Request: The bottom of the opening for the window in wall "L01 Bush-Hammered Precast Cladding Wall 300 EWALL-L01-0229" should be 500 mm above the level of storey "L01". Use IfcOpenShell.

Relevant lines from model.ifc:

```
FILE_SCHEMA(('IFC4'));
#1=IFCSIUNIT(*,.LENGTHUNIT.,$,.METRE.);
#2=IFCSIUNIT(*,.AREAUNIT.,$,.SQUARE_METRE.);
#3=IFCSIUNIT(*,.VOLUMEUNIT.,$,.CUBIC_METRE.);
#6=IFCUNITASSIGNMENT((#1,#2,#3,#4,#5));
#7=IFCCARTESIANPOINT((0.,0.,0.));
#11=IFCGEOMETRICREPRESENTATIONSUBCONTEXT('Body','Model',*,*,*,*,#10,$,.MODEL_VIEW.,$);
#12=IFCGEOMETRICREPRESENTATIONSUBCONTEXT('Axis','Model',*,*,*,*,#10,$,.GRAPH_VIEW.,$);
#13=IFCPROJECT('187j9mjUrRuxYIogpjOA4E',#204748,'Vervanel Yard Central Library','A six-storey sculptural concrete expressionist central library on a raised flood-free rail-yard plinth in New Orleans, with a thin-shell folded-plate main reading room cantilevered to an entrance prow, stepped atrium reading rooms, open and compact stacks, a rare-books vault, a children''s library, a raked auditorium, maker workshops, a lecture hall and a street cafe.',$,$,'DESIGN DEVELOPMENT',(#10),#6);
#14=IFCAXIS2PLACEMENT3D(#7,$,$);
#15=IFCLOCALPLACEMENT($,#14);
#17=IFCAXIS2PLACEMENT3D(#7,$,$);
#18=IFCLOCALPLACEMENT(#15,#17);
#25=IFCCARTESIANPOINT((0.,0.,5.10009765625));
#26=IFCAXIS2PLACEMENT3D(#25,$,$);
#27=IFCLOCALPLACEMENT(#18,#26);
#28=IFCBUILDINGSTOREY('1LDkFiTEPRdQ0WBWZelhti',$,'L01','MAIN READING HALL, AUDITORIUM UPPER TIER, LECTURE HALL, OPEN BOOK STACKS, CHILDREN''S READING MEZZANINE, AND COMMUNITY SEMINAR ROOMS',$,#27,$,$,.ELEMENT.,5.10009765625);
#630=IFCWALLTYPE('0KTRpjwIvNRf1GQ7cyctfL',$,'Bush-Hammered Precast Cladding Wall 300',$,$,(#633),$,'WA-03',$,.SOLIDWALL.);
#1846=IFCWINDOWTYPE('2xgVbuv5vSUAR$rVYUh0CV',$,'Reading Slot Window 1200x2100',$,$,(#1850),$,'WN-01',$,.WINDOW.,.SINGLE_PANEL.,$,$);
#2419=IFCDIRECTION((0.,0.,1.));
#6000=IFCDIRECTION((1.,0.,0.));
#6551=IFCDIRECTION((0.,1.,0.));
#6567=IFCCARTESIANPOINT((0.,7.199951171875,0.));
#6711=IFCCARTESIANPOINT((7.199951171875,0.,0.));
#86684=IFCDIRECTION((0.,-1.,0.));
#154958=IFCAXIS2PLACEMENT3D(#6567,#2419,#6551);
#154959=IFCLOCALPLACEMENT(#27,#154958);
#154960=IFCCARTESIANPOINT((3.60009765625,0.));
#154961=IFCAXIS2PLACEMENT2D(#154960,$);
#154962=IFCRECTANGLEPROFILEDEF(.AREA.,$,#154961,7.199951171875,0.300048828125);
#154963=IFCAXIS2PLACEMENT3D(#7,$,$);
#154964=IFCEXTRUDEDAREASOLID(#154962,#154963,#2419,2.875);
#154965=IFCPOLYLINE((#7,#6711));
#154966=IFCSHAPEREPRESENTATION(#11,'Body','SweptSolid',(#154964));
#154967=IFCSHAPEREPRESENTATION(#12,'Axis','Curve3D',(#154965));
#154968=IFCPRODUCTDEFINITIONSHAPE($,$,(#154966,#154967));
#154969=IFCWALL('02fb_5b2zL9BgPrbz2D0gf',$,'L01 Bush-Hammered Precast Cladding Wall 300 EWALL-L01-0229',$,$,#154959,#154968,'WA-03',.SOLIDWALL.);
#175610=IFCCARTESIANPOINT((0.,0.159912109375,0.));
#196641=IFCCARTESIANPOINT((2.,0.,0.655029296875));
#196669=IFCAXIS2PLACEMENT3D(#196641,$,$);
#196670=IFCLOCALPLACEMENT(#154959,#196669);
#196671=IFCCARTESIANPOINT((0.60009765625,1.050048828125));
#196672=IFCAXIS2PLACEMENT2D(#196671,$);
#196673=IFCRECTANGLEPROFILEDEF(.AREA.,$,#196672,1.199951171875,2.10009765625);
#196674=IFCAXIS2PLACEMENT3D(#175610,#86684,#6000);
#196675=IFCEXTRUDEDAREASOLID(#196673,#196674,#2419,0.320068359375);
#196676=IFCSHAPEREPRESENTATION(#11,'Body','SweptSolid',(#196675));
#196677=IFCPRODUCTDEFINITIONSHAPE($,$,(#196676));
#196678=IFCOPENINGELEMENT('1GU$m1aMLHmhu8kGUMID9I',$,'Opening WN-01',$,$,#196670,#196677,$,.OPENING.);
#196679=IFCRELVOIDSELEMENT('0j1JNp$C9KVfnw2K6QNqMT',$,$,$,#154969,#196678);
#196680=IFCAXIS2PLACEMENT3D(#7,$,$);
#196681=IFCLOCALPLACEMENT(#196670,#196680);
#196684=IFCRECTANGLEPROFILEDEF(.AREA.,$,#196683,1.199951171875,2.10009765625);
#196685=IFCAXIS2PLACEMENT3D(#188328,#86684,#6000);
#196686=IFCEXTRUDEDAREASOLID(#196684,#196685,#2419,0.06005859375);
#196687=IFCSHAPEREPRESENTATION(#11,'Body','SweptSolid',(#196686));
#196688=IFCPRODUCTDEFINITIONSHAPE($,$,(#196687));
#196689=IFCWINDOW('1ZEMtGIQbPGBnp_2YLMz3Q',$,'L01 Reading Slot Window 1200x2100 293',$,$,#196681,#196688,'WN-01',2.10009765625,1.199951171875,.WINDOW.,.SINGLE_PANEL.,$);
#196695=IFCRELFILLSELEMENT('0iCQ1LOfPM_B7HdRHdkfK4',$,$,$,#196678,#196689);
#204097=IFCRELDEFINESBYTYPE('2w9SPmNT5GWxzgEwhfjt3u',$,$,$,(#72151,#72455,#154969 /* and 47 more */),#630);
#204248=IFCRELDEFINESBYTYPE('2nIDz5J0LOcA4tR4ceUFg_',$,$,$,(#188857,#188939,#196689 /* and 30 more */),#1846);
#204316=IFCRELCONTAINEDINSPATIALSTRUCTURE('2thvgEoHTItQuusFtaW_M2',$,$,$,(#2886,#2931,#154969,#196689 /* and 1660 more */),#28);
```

```python
import numpy as np
import ifcopenshell
import ifcopenshell.api.geometry
import ifcopenshell.geom
import ifcopenshell.util.element
import ifcopenshell.util.placement
import ifcopenshell.util.shape
import ifcopenshell.util.unit

model = ifcopenshell.open("model.ifc")
unit_scale = ifcopenshell.util.unit.calculate_unit_scale(model)

window = model.by_guid("1ZEMtGIQbPGBnp_2YLMz3Q")
opening = window.FillsVoids[0].RelatingOpeningElement
storey = ifcopenshell.util.element.get_container(window, ifc_class="IfcBuildingStorey")
level = ifcopenshell.util.placement.get_local_placement(storey.ObjectPlacement)[2, 3]

# The opening's origin need not be at the sill, so measure its lowest point.
shape = ifcopenshell.geom.create_shape(ifcopenshell.geom.settings(), opening)
bottom = ifcopenshell.util.shape.get_shape_bottom_elevation(shape, shape.geometry) / unit_scale
dz = level + 0.5 / unit_scale - bottom

shift = np.array([0.0, 0.0, dz])
# The window is placed relative to its opening, so it follows when the opening moves.
matrix = ifcopenshell.util.placement.get_local_placement(opening.ObjectPlacement)
matrix[:3, 3] += shift
ifcopenshell.api.geometry.edit_object_placement(
    model, product=opening, matrix=matrix, is_si=False, should_transform_children=True
)

print(f"moved by {dz * unit_scale:+.3f} m")

model.write("model_rev.ifc")
```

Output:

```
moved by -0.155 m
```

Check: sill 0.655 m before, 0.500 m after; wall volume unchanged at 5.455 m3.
